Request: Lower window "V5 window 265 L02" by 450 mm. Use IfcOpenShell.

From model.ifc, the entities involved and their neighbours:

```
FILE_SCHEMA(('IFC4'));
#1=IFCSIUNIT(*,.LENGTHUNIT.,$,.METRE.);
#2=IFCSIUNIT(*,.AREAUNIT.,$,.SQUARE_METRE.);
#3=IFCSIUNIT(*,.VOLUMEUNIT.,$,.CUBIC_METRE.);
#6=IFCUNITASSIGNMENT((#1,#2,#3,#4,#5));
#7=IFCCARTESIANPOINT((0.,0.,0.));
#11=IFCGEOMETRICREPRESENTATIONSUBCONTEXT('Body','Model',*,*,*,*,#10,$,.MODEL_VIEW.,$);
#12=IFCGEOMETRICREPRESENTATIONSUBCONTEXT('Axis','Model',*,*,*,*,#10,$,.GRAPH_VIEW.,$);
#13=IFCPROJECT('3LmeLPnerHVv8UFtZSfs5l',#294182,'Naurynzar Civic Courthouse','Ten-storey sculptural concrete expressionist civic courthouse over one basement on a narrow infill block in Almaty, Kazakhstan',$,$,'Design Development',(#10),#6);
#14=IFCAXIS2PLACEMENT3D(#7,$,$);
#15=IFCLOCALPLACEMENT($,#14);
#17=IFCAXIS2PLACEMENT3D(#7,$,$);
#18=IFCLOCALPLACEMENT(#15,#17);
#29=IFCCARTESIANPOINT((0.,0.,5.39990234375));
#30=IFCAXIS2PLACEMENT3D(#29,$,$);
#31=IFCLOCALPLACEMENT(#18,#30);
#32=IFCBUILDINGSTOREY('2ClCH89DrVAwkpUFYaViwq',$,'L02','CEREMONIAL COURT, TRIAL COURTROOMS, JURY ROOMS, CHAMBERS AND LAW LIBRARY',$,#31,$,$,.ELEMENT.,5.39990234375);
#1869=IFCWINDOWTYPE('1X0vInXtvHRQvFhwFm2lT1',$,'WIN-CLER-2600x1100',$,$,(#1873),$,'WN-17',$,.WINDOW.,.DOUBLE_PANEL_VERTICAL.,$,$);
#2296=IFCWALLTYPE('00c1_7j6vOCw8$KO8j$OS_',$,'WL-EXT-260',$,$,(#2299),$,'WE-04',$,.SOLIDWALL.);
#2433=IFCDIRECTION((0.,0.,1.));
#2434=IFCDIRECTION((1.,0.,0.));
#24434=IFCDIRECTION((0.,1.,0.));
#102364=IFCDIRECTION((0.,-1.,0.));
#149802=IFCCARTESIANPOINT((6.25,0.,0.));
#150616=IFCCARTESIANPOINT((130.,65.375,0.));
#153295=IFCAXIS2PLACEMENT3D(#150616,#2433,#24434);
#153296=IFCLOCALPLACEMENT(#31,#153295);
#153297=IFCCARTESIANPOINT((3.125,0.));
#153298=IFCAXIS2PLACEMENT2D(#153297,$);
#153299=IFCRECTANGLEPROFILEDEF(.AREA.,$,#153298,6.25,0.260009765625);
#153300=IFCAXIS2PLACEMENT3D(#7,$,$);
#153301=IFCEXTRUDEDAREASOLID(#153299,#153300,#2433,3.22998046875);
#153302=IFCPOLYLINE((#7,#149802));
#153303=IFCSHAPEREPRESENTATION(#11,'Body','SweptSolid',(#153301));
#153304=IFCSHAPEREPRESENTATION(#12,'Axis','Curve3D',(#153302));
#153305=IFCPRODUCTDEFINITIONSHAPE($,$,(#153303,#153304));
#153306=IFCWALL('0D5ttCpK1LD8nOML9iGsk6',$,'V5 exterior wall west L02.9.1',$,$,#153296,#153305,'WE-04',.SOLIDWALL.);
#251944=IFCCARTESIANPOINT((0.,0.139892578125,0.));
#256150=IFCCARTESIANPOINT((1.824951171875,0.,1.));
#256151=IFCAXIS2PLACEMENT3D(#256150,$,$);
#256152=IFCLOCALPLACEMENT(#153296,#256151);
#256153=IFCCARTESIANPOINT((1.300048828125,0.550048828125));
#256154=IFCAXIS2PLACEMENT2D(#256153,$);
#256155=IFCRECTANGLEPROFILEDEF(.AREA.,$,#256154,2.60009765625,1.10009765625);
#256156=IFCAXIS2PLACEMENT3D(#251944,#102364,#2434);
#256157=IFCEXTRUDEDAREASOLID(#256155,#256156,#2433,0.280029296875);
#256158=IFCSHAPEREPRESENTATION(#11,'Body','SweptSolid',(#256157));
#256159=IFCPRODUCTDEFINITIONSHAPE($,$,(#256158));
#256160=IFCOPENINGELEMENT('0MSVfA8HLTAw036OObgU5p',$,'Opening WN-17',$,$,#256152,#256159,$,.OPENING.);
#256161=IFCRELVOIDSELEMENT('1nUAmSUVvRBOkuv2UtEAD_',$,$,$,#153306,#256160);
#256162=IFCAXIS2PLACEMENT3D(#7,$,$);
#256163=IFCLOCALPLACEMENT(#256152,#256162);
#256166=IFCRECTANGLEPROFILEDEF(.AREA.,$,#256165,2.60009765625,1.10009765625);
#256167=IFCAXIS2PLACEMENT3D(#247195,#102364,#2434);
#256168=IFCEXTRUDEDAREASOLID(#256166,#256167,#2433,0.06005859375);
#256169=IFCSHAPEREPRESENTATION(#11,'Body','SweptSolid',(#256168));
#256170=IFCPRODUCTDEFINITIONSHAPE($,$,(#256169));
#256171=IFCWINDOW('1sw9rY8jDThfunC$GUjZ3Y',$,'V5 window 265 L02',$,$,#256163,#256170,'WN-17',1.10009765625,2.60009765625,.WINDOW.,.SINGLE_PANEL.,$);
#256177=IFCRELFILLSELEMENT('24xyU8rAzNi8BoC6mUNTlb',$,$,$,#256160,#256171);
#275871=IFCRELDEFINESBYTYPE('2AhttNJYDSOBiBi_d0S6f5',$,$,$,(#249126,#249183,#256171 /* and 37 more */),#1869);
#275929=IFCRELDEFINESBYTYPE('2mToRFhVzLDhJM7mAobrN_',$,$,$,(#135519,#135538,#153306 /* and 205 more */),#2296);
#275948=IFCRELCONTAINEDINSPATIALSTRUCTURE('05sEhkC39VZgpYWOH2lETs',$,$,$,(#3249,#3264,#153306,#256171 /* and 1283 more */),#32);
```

```python
import numpy as np
import ifcopenshell
import ifcopenshell.api.geometry
import ifcopenshell.util.placement
import ifcopenshell.util.unit

model = ifcopenshell.open("model.ifc")
unit_scale = ifcopenshell.util.unit.calculate_unit_scale(model)

window = model.by_id(256171)
opening = window.FillsVoids[0].RelatingOpeningElement
dz = -0.45 / unit_scale

shift = np.array([0.0, 0.0, dz])
# The window is placed relative to its opening, so it follows when the opening moves.
matrix = ifcopenshell.util.placement.get_local_placement(opening.ObjectPlacement)
matrix[:3, 3] += shift
ifcopenshell.api.geometry.edit_object_placement(
    model, product=opening, matrix=matrix, is_si=False, should_transform_children=True
)

print(f"moved by {dz * unit_scale:+.3f} m")

model.write("model_v2.ifc")
```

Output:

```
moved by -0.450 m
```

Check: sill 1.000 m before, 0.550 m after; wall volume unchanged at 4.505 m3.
